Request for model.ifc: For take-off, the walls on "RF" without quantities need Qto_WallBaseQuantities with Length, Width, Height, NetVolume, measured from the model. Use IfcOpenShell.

First a look at what the model holds.

```python
import ifcopenshell
import ifcopenshell.util.element
import ifcopenshell.util.unit

model = ifcopenshell.open("model.ifc")
print(model.schema)
for unit_type in ("LENGTHUNIT", "AREAUNIT", "VOLUMEUNIT"):
    print(unit_type, ifcopenshell.util.unit.calculate_unit_scale(model, unit_type))
storey = next(s for s in model.by_type("IfcBuildingStorey") if s.Name == "RF")
walls = [e for e in ifcopenshell.util.element.get_decomposition(storey) if e.is_a("IfcWall")]
for e in sorted(walls, key=lambda e: e.id()):
    print(e.id(), e.is_a(), e.Name, list(ifcopenshell.util.element.get_psets(e, qtos_only=True)), sep=" | ")
```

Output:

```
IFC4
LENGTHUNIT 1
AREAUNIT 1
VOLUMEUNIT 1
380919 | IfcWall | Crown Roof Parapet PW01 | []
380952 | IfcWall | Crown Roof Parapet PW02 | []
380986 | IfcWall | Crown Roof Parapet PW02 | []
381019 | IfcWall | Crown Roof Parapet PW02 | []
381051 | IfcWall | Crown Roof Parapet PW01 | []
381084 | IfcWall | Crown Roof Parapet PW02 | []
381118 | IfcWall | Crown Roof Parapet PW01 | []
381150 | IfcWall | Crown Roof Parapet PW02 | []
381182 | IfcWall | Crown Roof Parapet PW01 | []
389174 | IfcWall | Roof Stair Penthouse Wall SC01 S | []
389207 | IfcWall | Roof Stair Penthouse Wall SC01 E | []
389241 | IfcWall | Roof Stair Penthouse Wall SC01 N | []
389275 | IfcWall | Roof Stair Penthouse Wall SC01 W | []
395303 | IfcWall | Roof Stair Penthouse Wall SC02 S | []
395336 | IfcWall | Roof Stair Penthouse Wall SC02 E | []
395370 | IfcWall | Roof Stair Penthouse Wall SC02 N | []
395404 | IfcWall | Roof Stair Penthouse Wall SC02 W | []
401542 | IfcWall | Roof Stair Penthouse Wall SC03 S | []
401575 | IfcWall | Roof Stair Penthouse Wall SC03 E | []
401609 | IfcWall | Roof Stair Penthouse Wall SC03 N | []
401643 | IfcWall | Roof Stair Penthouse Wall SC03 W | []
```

```python
import ifcopenshell
import ifcopenshell.api.pset
import ifcopenshell.geom
import ifcopenshell.util.element
import ifcopenshell.util.shape
import ifcopenshell.util.unit

model = ifcopenshell.open("model.ifc")
unit_scale = ifcopenshell.util.unit.calculate_unit_scale(model)
volume_scale = ifcopenshell.util.unit.calculate_unit_scale(model, "VOLUMEUNIT")
settings = ifcopenshell.geom.settings()

storey = next(s for s in model.by_type("IfcBuildingStorey") if s.Name == "RF")
walls = [e for e in ifcopenshell.util.element.get_decomposition(storey) if e.is_a("IfcWall")]

for e in sorted(walls, key=lambda e: e.id()):
    if ifcopenshell.util.element.get_psets(e, qtos_only=True, should_inherit=False):
        continue
    # Geometry comes back in metres, in the element's own axes.
    shape = ifcopenshell.geom.create_shape(settings, e)
    values = {
        "Length": ifcopenshell.util.shape.get_x(shape.geometry) / unit_scale,
        "Width": ifcopenshell.util.shape.get_y(shape.geometry) / unit_scale,
        "Height": ifcopenshell.util.shape.get_z(shape.geometry) / unit_scale,
        "NetVolume": ifcopenshell.util.shape.get_volume(shape.geometry) / volume_scale,
    }
    qto = ifcopenshell.api.pset.add_qto(model, product=e, name="Qto_WallBaseQuantities")
    ifcopenshell.api.pset.edit_qto(model, qto=qto, properties=values)
    print(e.id(), {k: round(v, 3) for k, v in values.items()})

model.write("model_v2.ifc")
```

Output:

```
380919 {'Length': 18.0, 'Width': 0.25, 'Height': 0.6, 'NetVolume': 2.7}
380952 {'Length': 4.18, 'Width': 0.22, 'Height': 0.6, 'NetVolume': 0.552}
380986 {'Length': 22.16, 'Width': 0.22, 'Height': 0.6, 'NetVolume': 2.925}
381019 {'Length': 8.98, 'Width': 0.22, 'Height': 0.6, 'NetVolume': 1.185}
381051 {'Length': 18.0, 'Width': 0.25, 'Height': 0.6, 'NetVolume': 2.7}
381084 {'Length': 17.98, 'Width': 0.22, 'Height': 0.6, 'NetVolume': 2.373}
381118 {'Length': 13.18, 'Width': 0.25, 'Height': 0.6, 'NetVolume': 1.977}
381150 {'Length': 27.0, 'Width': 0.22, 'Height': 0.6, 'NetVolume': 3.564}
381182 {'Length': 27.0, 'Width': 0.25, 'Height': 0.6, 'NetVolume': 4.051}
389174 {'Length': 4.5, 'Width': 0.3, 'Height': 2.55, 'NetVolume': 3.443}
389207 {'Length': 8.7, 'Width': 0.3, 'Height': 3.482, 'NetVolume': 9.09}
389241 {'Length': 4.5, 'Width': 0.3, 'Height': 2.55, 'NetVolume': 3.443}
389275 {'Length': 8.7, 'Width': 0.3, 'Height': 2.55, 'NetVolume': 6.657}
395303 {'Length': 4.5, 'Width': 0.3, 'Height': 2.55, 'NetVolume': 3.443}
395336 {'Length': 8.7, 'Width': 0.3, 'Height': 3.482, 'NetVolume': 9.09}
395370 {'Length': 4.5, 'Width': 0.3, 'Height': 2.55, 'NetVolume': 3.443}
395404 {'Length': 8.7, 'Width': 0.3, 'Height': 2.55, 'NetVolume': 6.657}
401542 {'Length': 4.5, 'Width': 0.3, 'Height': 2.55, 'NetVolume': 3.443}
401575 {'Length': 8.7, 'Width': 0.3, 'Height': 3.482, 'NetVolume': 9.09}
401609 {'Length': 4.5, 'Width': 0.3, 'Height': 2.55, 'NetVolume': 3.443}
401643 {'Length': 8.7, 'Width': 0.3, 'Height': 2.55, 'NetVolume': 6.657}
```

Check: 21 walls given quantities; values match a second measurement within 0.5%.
